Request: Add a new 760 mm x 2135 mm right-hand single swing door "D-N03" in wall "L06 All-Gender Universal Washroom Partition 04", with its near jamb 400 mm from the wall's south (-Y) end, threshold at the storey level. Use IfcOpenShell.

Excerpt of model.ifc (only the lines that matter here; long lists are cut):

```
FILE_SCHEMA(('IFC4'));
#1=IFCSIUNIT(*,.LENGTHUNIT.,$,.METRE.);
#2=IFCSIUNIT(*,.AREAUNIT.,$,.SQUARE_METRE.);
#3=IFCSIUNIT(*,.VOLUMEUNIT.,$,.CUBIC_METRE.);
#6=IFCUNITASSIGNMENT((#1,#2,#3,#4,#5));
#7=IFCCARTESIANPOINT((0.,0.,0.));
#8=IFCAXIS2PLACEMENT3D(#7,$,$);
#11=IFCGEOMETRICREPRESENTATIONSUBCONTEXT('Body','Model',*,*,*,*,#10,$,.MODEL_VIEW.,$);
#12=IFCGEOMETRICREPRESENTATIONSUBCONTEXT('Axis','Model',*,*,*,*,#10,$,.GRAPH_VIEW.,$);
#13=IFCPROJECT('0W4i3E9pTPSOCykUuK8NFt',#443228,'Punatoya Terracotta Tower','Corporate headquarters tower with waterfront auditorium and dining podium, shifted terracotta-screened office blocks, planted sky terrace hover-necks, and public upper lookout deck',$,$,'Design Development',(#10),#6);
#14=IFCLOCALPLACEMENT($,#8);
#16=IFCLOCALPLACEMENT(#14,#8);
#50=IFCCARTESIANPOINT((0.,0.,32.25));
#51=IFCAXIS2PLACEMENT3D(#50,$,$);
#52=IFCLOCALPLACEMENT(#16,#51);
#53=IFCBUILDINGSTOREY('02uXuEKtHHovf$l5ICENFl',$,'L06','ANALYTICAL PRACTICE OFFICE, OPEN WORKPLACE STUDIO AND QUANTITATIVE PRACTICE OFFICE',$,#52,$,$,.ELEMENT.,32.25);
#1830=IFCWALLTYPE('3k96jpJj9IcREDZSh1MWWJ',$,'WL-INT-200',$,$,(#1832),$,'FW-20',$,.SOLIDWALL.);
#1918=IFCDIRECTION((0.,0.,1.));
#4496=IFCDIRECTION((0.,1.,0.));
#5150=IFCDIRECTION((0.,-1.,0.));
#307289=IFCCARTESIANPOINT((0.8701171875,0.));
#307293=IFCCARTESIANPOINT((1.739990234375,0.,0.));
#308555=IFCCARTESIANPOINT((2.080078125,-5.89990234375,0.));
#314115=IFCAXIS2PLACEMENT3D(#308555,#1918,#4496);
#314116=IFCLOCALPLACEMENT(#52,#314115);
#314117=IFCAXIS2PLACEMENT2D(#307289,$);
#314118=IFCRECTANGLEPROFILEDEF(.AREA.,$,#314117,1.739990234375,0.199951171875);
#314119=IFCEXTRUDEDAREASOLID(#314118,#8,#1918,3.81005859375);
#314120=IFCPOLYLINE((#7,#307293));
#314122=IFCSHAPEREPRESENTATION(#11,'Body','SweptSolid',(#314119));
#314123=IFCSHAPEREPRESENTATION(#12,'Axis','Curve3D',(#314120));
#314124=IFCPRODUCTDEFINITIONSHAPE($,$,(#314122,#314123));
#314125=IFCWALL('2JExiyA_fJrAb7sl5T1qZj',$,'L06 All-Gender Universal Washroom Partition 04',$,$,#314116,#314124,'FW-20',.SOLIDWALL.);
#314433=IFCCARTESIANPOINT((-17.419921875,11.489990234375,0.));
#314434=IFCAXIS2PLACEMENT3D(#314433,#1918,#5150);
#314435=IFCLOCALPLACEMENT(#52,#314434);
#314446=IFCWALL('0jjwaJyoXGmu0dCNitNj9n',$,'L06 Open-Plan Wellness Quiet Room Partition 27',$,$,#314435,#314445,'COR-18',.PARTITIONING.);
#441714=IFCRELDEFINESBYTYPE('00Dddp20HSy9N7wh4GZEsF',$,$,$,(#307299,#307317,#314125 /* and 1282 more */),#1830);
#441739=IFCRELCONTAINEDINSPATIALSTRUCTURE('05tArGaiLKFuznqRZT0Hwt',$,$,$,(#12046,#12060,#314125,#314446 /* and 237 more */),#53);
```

```python
import numpy as np
import ifcopenshell
import ifcopenshell.api.feature
import ifcopenshell.api.geometry
import ifcopenshell.api.root
import ifcopenshell.api.spatial
import ifcopenshell.geom
import ifcopenshell.util.element
import ifcopenshell.util.placement
import ifcopenshell.util.representation
import ifcopenshell.util.shape
import ifcopenshell.util.unit

model = ifcopenshell.open("model.ifc")
unit_scale = ifcopenshell.util.unit.calculate_unit_scale(model)
settings = ifcopenshell.geom.settings()


def volume(element):
    """Net volume in cubic metres, openings subtracted."""
    shape = ifcopenshell.geom.create_shape(settings, element)
    return ifcopenshell.util.shape.get_volume(shape.geometry)


wall = model.by_id(314125)
storey = ifcopenshell.util.element.get_container(wall, ifc_class="IfcBuildingStorey")
context = ifcopenshell.util.representation.get_context(model, "Model", "Body", "MODEL_VIEW")
before = volume(wall)

width, height, from_end, sill = 0.76, 2.135, 0.4, 0.0  # metres

# The wall runs along its own X axis, and the end named is its -X end.
wall_shape = ifcopenshell.geom.create_shape(settings, wall)
x, y, z = ifcopenshell.util.shape.get_vertices(wall_shape.geometry).T
start = x.min() + from_end
face, thickness = float(y.min()), float(y.max() - y.min())
wall_matrix = ifcopenshell.util.placement.get_local_placement(wall.ObjectPlacement)
level = ifcopenshell.util.placement.get_local_placement(storey.ObjectPlacement)[2, 3]


def in_wall(x, y):
    """Placement at x, y metres in the wall's axes, at sill height."""
    matrix = wall_matrix.copy()
    matrix[:, 3] = wall_matrix @ np.array([x / unit_scale, y / unit_scale, 0.0, 1.0])
    matrix[2, 3] = level + sill / unit_scale
    return matrix


# Opening: a box that overshoots both wall faces by 50 mm.
opening = ifcopenshell.api.root.create_entity(model, ifc_class="IfcOpeningElement", predefined_type="OPENING")
box = ifcopenshell.api.geometry.add_wall_representation(
    model, context=context, length=width, height=height, thickness=thickness + 0.1
)
ifcopenshell.api.geometry.assign_representation(model, product=opening, representation=box)
ifcopenshell.api.geometry.edit_object_placement(model, product=opening, matrix=in_wall(start, face - 0.05), is_si=False)
ifcopenshell.api.feature.add_feature(model, feature=opening, element=wall)

door = ifcopenshell.api.root.create_entity(model, ifc_class="IfcDoor", name="D-N03", predefined_type="DOOR")
door.OverallWidth, door.OverallHeight = width / unit_scale, height / unit_scale
door.OperationType = "SINGLE_SWING_RIGHT"
body = ifcopenshell.api.geometry.add_door_representation(
    model,
    context=context,
    overall_width=door.OverallWidth,
    overall_height=door.OverallHeight,
    operation_type="SINGLE_SWING_RIGHT",
    lining_properties={"LiningDepth": thickness / unit_scale, "ThresholdDepth": thickness / unit_scale},
)
ifcopenshell.api.geometry.assign_representation(model, product=door, representation=body)
ifcopenshell.api.spatial.assign_container(model, products=[door], relating_structure=storey)
ifcopenshell.api.feature.add_filling(model, opening=opening, element=door)

# The lining spans the wall, so the door starts at the wall face.
ifcopenshell.api.geometry.edit_object_placement(model, product=door, matrix=in_wall(start, face), is_si=False)

after = volume(wall)

print(f"wall volume {before:.3f} -> {after:.3f} m3")

model.write("model-out.ifc")
```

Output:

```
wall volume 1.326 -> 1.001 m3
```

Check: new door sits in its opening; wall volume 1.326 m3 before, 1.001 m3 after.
